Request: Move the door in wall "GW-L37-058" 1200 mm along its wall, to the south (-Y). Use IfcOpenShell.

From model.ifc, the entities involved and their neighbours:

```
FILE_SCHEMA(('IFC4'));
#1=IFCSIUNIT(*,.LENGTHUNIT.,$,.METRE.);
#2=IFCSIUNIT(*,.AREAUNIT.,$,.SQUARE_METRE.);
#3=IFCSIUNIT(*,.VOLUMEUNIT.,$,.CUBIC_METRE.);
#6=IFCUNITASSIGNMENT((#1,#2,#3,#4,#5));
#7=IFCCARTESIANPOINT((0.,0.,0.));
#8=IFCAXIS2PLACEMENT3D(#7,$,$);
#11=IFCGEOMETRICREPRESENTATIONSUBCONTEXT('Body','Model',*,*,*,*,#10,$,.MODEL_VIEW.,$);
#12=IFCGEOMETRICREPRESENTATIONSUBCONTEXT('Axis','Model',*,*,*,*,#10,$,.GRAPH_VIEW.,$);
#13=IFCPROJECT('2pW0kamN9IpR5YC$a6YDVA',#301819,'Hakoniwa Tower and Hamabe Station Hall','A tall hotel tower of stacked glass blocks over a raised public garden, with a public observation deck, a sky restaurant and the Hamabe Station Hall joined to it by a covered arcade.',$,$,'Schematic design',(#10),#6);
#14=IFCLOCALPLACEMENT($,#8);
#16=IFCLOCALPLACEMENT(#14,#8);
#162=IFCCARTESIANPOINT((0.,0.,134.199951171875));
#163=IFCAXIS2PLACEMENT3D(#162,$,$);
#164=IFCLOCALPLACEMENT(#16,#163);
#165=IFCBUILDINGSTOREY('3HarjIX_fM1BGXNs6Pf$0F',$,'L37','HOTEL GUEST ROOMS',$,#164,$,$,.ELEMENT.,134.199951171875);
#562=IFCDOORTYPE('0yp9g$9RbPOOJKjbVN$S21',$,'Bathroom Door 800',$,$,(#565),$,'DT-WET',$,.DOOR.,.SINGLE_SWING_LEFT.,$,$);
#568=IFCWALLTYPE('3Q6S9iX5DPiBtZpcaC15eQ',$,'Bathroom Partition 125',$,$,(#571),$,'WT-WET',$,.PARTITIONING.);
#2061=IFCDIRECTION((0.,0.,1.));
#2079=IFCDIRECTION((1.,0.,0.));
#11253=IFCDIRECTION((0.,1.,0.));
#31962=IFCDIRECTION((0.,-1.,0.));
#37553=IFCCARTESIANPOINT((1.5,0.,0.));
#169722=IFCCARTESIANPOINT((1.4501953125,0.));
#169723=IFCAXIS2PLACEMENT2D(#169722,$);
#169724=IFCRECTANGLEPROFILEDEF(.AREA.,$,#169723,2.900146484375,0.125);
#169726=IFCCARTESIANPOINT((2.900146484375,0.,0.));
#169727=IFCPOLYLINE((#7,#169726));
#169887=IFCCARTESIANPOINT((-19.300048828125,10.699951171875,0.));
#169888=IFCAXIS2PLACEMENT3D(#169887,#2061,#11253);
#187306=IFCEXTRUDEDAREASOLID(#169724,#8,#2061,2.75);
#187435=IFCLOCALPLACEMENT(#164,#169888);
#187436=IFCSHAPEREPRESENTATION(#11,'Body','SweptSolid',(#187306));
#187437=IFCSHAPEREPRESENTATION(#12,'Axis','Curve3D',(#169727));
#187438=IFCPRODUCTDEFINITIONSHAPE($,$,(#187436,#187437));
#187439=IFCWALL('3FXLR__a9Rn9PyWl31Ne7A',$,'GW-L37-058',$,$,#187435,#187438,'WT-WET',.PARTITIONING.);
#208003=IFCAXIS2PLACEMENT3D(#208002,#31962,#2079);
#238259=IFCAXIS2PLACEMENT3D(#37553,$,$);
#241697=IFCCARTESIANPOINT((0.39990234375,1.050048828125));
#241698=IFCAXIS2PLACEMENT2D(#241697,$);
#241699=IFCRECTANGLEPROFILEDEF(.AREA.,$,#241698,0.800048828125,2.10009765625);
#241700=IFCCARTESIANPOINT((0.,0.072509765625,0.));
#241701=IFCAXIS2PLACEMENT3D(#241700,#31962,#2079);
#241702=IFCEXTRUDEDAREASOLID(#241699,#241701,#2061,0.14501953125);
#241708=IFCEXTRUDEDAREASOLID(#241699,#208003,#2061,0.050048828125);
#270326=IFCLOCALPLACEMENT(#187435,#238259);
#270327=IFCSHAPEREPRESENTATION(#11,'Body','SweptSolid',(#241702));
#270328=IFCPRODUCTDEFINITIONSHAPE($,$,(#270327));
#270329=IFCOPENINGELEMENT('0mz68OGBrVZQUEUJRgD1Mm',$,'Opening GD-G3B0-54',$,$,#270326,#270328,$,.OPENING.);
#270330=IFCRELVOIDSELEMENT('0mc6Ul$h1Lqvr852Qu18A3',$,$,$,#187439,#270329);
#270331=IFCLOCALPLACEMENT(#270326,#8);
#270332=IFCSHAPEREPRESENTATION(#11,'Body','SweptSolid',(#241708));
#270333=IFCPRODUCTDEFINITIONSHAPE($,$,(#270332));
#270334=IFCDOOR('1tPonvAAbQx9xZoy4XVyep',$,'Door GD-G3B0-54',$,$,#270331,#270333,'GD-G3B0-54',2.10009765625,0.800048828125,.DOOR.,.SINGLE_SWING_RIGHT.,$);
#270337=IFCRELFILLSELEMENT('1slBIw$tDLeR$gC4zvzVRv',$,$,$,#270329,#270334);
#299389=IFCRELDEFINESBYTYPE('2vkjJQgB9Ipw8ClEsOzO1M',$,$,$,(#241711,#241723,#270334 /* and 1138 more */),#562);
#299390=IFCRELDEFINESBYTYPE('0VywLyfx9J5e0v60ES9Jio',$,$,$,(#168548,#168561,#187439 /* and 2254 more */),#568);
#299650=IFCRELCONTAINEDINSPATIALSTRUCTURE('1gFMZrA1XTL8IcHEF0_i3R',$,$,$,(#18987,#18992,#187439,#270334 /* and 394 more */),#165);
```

```python
import ifcopenshell
import ifcopenshell.api.geometry
import ifcopenshell.util.placement

model = ifcopenshell.open("model.ifc")

door = model.by_guid("1tPonvAAbQx9xZoy4XVyep")
opening = door.FillsVoids[0].RelatingOpeningElement
wall = opening.VoidsElements[0].RelatingBuildingElement

wall_matrix = ifcopenshell.util.placement.get_local_placement(wall.ObjectPlacement)
shift = wall_matrix[:3, 0] * -1.2
before = ifcopenshell.util.placement.get_local_placement(door.ObjectPlacement)[:3, 3].copy()

# The door is placed relative to its opening, so it follows when the opening moves.
matrix = ifcopenshell.util.placement.get_local_placement(opening.ObjectPlacement)
matrix[:3, 3] += shift
ifcopenshell.api.geometry.edit_object_placement(
    model, product=opening, matrix=matrix, is_si=False, should_transform_children=True
)

after = ifcopenshell.util.placement.get_local_placement(door.ObjectPlacement)[:3, 3]
print("door moved by", (after - before).round(3) + 0.0)

model.write("model_edited.ifc")
```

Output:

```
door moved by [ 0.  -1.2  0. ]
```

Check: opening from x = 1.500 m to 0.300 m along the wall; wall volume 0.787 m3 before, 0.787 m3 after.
